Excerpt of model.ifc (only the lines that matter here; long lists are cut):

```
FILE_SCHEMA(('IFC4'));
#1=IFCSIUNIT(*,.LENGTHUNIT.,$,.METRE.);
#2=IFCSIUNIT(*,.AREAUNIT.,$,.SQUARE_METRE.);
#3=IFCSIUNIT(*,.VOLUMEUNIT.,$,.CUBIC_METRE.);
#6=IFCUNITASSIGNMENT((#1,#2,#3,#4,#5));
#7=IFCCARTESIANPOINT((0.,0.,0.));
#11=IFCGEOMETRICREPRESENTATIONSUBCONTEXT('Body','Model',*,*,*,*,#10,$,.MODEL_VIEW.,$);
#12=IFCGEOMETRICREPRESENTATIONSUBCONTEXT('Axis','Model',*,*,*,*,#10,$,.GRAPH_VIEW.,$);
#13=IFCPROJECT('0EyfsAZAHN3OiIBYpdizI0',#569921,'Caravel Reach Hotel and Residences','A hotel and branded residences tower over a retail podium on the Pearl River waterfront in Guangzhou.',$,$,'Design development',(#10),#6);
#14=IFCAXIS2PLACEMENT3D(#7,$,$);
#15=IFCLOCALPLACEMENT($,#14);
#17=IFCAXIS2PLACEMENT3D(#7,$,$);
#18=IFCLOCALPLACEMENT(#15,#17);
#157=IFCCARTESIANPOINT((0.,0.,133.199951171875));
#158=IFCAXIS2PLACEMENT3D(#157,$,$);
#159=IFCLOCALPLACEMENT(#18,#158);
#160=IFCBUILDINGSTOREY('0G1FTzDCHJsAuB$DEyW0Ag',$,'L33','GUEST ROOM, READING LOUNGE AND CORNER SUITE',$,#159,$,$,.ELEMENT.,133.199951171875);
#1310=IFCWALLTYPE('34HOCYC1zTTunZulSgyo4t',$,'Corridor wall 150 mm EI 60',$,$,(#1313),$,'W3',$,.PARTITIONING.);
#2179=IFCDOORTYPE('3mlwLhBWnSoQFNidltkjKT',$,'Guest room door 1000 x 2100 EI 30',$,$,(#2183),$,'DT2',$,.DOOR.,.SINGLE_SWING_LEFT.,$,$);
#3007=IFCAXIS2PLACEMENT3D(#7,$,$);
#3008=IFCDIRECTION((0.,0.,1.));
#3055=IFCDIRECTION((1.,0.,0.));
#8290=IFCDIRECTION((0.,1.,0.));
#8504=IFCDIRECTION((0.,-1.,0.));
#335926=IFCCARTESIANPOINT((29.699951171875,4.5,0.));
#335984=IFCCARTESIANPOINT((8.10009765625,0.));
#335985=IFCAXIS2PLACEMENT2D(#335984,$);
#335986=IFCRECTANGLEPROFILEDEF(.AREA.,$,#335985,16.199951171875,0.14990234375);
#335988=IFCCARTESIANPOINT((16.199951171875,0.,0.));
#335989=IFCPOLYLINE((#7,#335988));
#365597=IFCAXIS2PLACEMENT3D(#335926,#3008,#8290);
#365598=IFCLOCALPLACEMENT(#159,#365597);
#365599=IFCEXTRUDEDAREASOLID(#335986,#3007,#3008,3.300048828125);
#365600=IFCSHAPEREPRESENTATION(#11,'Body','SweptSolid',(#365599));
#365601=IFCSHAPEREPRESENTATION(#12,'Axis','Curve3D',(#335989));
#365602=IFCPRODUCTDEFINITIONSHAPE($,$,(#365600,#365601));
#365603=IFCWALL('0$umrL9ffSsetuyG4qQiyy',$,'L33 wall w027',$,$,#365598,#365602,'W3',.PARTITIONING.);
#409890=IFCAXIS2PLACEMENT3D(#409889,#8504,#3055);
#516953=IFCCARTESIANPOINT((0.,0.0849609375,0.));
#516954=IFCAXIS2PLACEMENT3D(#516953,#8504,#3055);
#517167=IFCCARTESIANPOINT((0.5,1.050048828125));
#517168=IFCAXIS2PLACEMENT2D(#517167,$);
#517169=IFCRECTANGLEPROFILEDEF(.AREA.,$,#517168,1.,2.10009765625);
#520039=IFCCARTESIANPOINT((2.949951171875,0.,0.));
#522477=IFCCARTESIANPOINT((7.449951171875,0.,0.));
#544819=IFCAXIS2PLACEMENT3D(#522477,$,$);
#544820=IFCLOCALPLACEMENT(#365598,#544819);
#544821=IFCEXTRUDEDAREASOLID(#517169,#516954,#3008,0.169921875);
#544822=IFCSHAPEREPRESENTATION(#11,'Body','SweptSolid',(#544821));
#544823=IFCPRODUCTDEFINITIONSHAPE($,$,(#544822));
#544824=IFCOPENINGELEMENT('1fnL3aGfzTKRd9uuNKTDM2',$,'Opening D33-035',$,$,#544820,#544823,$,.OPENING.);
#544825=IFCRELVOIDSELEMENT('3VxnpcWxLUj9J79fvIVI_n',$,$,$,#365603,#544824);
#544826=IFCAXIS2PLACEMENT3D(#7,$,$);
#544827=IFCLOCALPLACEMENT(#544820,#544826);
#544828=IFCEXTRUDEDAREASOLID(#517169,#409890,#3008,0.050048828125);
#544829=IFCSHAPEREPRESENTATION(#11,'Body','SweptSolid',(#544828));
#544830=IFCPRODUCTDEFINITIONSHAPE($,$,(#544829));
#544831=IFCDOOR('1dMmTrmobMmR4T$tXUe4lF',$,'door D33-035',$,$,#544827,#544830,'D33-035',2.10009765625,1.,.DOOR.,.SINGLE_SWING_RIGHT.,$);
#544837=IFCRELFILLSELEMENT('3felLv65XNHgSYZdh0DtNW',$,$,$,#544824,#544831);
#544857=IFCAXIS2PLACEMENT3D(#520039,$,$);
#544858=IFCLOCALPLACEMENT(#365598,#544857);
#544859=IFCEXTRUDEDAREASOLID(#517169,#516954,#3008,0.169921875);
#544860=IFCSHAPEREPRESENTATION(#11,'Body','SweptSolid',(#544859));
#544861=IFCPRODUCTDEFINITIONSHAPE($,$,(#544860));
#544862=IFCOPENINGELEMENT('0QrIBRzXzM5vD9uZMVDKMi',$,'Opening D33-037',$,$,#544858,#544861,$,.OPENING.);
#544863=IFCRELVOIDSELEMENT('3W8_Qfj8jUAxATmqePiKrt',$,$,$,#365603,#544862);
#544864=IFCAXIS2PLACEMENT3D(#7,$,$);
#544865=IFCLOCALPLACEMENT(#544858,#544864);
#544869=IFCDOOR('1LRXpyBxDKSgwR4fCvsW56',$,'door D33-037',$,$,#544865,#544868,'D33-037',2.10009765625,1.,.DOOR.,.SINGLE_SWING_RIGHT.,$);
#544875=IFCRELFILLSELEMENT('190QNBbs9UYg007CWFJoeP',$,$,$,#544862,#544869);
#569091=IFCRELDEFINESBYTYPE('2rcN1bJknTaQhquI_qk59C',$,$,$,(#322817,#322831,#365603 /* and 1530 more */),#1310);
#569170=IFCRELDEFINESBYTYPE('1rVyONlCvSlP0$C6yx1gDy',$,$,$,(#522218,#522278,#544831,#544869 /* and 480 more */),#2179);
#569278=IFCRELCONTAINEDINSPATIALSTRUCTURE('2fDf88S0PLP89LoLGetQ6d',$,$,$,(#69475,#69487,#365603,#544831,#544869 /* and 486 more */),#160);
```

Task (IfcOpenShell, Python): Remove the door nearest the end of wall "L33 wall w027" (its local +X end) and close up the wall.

```python
import ifcopenshell
import ifcopenshell.api.feature
import ifcopenshell.api.root
import ifcopenshell.geom
import ifcopenshell.util.shape

model = ifcopenshell.open("model.ifc")
settings = ifcopenshell.geom.settings()


def volume(element):
    """Net volume in cubic metres, openings subtracted."""
    shape = ifcopenshell.geom.create_shape(settings, element)
    return ifcopenshell.util.shape.get_volume(shape.geometry)


door = model.by_guid("1dMmTrmobMmR4T$tXUe4lF")
opening = door.FillsVoids[0].RelatingOpeningElement
wall = opening.VoidsElements[0].RelatingBuildingElement
before = volume(wall)

ifcopenshell.api.root.remove_product(model, product=door)
ifcopenshell.api.feature.remove_feature(model, feature=opening)

after = volume(wall)

print(f"wall volume {before:.3f} -> {after:.3f} m3")

model.write("model_updated.ifc")
```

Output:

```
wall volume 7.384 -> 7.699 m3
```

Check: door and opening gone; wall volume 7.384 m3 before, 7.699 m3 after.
